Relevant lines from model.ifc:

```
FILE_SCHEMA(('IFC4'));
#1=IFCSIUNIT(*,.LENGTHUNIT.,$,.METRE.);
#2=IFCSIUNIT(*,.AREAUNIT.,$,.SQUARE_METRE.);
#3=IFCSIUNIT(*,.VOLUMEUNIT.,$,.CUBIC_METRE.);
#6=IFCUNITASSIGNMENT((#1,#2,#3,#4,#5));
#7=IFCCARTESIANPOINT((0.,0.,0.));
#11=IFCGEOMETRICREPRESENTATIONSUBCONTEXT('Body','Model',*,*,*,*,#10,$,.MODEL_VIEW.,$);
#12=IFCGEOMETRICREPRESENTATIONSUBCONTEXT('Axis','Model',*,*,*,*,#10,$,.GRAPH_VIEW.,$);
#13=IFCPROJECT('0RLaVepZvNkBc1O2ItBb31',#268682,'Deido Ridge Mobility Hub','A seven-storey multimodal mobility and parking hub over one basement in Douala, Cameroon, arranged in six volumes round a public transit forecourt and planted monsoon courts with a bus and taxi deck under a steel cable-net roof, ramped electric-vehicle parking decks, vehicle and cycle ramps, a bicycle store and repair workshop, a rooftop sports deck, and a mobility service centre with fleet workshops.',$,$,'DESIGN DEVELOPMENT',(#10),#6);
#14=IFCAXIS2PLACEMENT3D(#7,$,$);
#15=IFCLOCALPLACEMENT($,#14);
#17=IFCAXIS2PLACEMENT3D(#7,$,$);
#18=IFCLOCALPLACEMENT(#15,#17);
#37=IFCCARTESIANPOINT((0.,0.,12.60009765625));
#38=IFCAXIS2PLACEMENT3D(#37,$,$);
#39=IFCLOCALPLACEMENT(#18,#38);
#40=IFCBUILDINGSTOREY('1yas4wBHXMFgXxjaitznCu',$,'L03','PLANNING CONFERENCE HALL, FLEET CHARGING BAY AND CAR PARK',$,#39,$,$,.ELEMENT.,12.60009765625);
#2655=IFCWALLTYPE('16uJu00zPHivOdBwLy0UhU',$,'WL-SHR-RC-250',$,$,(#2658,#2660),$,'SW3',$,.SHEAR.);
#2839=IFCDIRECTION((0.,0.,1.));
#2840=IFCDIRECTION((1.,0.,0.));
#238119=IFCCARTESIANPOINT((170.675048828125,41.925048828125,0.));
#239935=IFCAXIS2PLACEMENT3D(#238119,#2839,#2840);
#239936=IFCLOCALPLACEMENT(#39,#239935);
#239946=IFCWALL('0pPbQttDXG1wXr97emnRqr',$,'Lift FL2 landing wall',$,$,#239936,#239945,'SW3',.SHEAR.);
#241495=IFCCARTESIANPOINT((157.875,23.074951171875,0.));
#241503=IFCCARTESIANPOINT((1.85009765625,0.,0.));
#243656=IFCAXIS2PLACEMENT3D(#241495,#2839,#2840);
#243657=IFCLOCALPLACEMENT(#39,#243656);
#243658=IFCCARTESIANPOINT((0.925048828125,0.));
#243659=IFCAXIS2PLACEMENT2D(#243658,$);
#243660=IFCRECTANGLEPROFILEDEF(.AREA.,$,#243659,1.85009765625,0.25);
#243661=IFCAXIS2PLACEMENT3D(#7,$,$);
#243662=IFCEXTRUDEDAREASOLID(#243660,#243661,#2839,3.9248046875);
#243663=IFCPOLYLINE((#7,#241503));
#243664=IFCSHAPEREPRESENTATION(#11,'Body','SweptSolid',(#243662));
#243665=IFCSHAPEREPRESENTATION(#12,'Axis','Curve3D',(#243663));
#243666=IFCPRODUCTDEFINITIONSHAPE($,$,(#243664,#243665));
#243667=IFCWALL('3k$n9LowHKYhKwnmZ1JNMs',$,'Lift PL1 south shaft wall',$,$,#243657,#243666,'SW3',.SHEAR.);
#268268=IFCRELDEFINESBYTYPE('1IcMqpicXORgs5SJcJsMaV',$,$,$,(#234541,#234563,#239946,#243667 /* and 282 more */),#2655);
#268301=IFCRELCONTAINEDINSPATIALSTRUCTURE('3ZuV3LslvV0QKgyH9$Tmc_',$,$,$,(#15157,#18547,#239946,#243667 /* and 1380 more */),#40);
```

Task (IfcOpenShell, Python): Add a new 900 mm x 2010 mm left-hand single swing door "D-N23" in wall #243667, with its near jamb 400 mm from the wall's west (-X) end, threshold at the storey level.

```python
import numpy as np
import ifcopenshell
import ifcopenshell.api.feature
import ifcopenshell.api.geometry
import ifcopenshell.api.root
import ifcopenshell.api.spatial
import ifcopenshell.geom
import ifcopenshell.util.element
import ifcopenshell.util.placement
import ifcopenshell.util.representation
import ifcopenshell.util.shape
import ifcopenshell.util.unit

model = ifcopenshell.open("model.ifc")
unit_scale = ifcopenshell.util.unit.calculate_unit_scale(model)
settings = ifcopenshell.geom.settings()


def volume(element):
    """Net volume in cubic metres, openings subtracted."""
    shape = ifcopenshell.geom.create_shape(settings, element)
    return ifcopenshell.util.shape.get_volume(shape.geometry)


wall = model.by_id(243667)
storey = ifcopenshell.util.element.get_container(wall, ifc_class="IfcBuildingStorey")
context = ifcopenshell.util.representation.get_context(model, "Model", "Body", "MODEL_VIEW")
before = volume(wall)

width, height, from_end, sill = 0.9, 2.01, 0.4, 0.0  # metres

# The wall runs along its own X axis, and the end named is its -X end.
wall_shape = ifcopenshell.geom.create_shape(settings, wall)
x, y, z = ifcopenshell.util.shape.get_vertices(wall_shape.geometry).T
start = x.min() + from_end
face, thickness = float(y.min()), float(y.max() - y.min())
wall_matrix = ifcopenshell.util.placement.get_local_placement(wall.ObjectPlacement)
level = ifcopenshell.util.placement.get_local_placement(storey.ObjectPlacement)[2, 3]


def in_wall(x, y):
    """Placement at x, y metres in the wall's axes, at sill height."""
    matrix = wall_matrix.copy()
    matrix[:, 3] = wall_matrix @ np.array([x / unit_scale, y / unit_scale, 0.0, 1.0])
    matrix[2, 3] = level + sill / unit_scale
    return matrix


# Opening: a box that overshoots both wall faces by 50 mm.
opening = ifcopenshell.api.root.create_entity(model, ifc_class="IfcOpeningElement", predefined_type="OPENING")
box = ifcopenshell.api.geometry.add_wall_representation(
    model, context=context, length=width, height=height, thickness=thickness + 0.1
)
ifcopenshell.api.geometry.assign_representation(model, product=opening, representation=box)
ifcopenshell.api.geometry.edit_object_placement(model, product=opening, matrix=in_wall(start, face - 0.05), is_si=False)
ifcopenshell.api.feature.add_feature(model, feature=opening, element=wall)

door = ifcopenshell.api.root.create_entity(model, ifc_class="IfcDoor", name="D-N23", predefined_type="DOOR")
door.OverallWidth, door.OverallHeight = width / unit_scale, height / unit_scale
door.OperationType = "SINGLE_SWING_LEFT"
body = ifcopenshell.api.geometry.add_door_representation(
    model,
    context=context,
    overall_width=door.OverallWidth,
    overall_height=door.OverallHeight,
    operation_type="SINGLE_SWING_LEFT",
    lining_properties={"LiningDepth": thickness / unit_scale, "ThresholdDepth": thickness / unit_scale},
)
ifcopenshell.api.geometry.assign_representation(model, product=door, representation=body)
ifcopenshell.api.spatial.assign_container(model, products=[door], relating_structure=storey)
ifcopenshell.api.feature.add_filling(model, opening=opening, element=door)

# The lining spans the wall, so the door starts at the wall face.
ifcopenshell.api.geometry.edit_object_placement(model, product=door, matrix=in_wall(start, face), is_si=False)

after = volume(wall)

print(f"wall volume {before:.3f} -> {after:.3f} m3")

model.write("model_edited.ifc")
```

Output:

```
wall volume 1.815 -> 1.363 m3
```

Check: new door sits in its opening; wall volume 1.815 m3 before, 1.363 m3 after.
